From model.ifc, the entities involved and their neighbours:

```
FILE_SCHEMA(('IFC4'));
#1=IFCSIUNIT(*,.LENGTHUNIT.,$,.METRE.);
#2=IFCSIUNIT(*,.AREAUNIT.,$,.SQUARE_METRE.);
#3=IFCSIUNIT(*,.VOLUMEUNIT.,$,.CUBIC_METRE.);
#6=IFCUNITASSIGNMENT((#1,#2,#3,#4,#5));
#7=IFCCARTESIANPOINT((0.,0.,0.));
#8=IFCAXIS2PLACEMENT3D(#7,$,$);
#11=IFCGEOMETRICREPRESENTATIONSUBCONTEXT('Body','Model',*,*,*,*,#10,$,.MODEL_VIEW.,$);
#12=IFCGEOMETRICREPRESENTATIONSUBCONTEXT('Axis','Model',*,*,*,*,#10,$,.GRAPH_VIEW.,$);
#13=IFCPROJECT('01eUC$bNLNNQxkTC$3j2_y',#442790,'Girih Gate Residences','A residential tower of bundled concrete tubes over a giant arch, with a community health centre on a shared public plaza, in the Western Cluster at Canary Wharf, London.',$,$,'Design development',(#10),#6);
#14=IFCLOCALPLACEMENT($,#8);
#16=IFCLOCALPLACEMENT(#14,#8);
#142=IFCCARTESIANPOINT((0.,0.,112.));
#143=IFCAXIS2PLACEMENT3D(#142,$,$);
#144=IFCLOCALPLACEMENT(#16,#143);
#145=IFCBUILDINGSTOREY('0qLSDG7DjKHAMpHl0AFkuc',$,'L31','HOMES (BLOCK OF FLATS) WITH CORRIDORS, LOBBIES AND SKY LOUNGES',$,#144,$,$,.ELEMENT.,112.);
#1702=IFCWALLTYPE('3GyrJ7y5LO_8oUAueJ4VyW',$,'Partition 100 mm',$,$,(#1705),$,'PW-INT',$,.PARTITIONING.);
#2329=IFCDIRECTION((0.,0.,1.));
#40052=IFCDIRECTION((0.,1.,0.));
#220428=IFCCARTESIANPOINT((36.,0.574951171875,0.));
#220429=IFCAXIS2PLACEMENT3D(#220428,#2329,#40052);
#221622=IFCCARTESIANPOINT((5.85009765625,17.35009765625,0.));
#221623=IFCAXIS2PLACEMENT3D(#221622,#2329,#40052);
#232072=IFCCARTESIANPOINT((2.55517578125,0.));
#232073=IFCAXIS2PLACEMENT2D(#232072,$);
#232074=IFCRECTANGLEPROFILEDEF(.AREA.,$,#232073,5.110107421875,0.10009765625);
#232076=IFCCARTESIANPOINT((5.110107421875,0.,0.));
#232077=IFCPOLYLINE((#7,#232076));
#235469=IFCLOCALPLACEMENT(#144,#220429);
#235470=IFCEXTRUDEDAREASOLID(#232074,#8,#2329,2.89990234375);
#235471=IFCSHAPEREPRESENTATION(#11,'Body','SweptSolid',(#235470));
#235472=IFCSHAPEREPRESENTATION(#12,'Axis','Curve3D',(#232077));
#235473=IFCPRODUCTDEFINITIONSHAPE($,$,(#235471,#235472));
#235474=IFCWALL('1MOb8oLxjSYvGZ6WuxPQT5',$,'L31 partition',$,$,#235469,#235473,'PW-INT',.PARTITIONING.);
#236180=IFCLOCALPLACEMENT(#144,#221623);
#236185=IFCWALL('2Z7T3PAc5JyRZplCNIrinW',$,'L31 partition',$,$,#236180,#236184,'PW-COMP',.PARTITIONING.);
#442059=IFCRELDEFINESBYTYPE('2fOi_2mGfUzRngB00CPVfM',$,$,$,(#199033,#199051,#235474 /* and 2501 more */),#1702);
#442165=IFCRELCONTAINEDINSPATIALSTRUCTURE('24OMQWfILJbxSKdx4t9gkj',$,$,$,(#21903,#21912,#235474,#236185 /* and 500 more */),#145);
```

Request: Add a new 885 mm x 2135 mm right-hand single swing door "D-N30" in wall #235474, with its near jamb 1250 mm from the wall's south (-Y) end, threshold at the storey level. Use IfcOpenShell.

```python
import numpy as np
import ifcopenshell
import ifcopenshell.api.feature
import ifcopenshell.api.geometry
import ifcopenshell.api.root
import ifcopenshell.api.spatial
import ifcopenshell.geom
import ifcopenshell.util.element
import ifcopenshell.util.placement
import ifcopenshell.util.representation
import ifcopenshell.util.shape
import ifcopenshell.util.unit

model = ifcopenshell.open("model.ifc")
unit_scale = ifcopenshell.util.unit.calculate_unit_scale(model)
settings = ifcopenshell.geom.settings()


def volume(element):
    """Net volume in cubic metres, openings subtracted."""
    shape = ifcopenshell.geom.create_shape(settings, element)
    return ifcopenshell.util.shape.get_volume(shape.geometry)


wall = model.by_id(235474)
storey = ifcopenshell.util.element.get_container(wall, ifc_class="IfcBuildingStorey")
context = ifcopenshell.util.representation.get_context(model, "Model", "Body", "MODEL_VIEW")
before = volume(wall)

width, height, from_end, sill = 0.885, 2.135, 1.25, 0.0  # metres

# The wall runs along its own X axis, and the end named is its -X end.
wall_shape = ifcopenshell.geom.create_shape(settings, wall)
x, y, z = ifcopenshell.util.shape.get_vertices(wall_shape.geometry).T
start = x.min() + from_end
face, thickness = float(y.min()), float(y.max() - y.min())
wall_matrix = ifcopenshell.util.placement.get_local_placement(wall.ObjectPlacement)
level = ifcopenshell.util.placement.get_local_placement(storey.ObjectPlacement)[2, 3]


def in_wall(x, y):
    """Placement at x, y metres in the wall's axes, at sill height."""
    matrix = wall_matrix.copy()
    matrix[:, 3] = wall_matrix @ np.array([x / unit_scale, y / unit_scale, 0.0, 1.0])
    matrix[2, 3] = level + sill / unit_scale
    return matrix


# Opening: a box that overshoots both wall faces by 50 mm.
opening = ifcopenshell.api.root.create_entity(model, ifc_class="IfcOpeningElement", predefined_type="OPENING")
box = ifcopenshell.api.geometry.add_wall_representation(
    model, context=context, length=width, height=height, thickness=thickness + 0.1
)
ifcopenshell.api.geometry.assign_representation(model, product=opening, representation=box)
ifcopenshell.api.geometry.edit_object_placement(model, product=opening, matrix=in_wall(start, face - 0.05), is_si=False)
ifcopenshell.api.feature.add_feature(model, feature=opening, element=wall)

door = ifcopenshell.api.root.create_entity(model, ifc_class="IfcDoor", name="D-N30", predefined_type="DOOR")
door.OverallWidth, door.OverallHeight = width / unit_scale, height / unit_scale
door.OperationType = "SINGLE_SWING_RIGHT"
body = ifcopenshell.api.geometry.add_door_representation(
    model,
    context=context,
    overall_width=door.OverallWidth,
    overall_height=door.OverallHeight,
    operation_type="SINGLE_SWING_RIGHT",
    lining_properties={"LiningDepth": thickness / unit_scale, "ThresholdDepth": thickness / unit_scale},
)
ifcopenshell.api.geometry.assign_representation(model, product=door, representation=body)
ifcopenshell.api.spatial.assign_container(model, products=[door], relating_structure=storey)
ifcopenshell.api.feature.add_filling(model, opening=opening, element=door)

# The lining spans the wall, so the door starts at the wall face.
ifcopenshell.api.geometry.edit_object_placement(model, product=door, matrix=in_wall(start, face), is_si=False)

after = volume(wall)

print(f"wall volume {before:.3f} -> {after:.3f} m3")

model.write("model_v2.ifc")
```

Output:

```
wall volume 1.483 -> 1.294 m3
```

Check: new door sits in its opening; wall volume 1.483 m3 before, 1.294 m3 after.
